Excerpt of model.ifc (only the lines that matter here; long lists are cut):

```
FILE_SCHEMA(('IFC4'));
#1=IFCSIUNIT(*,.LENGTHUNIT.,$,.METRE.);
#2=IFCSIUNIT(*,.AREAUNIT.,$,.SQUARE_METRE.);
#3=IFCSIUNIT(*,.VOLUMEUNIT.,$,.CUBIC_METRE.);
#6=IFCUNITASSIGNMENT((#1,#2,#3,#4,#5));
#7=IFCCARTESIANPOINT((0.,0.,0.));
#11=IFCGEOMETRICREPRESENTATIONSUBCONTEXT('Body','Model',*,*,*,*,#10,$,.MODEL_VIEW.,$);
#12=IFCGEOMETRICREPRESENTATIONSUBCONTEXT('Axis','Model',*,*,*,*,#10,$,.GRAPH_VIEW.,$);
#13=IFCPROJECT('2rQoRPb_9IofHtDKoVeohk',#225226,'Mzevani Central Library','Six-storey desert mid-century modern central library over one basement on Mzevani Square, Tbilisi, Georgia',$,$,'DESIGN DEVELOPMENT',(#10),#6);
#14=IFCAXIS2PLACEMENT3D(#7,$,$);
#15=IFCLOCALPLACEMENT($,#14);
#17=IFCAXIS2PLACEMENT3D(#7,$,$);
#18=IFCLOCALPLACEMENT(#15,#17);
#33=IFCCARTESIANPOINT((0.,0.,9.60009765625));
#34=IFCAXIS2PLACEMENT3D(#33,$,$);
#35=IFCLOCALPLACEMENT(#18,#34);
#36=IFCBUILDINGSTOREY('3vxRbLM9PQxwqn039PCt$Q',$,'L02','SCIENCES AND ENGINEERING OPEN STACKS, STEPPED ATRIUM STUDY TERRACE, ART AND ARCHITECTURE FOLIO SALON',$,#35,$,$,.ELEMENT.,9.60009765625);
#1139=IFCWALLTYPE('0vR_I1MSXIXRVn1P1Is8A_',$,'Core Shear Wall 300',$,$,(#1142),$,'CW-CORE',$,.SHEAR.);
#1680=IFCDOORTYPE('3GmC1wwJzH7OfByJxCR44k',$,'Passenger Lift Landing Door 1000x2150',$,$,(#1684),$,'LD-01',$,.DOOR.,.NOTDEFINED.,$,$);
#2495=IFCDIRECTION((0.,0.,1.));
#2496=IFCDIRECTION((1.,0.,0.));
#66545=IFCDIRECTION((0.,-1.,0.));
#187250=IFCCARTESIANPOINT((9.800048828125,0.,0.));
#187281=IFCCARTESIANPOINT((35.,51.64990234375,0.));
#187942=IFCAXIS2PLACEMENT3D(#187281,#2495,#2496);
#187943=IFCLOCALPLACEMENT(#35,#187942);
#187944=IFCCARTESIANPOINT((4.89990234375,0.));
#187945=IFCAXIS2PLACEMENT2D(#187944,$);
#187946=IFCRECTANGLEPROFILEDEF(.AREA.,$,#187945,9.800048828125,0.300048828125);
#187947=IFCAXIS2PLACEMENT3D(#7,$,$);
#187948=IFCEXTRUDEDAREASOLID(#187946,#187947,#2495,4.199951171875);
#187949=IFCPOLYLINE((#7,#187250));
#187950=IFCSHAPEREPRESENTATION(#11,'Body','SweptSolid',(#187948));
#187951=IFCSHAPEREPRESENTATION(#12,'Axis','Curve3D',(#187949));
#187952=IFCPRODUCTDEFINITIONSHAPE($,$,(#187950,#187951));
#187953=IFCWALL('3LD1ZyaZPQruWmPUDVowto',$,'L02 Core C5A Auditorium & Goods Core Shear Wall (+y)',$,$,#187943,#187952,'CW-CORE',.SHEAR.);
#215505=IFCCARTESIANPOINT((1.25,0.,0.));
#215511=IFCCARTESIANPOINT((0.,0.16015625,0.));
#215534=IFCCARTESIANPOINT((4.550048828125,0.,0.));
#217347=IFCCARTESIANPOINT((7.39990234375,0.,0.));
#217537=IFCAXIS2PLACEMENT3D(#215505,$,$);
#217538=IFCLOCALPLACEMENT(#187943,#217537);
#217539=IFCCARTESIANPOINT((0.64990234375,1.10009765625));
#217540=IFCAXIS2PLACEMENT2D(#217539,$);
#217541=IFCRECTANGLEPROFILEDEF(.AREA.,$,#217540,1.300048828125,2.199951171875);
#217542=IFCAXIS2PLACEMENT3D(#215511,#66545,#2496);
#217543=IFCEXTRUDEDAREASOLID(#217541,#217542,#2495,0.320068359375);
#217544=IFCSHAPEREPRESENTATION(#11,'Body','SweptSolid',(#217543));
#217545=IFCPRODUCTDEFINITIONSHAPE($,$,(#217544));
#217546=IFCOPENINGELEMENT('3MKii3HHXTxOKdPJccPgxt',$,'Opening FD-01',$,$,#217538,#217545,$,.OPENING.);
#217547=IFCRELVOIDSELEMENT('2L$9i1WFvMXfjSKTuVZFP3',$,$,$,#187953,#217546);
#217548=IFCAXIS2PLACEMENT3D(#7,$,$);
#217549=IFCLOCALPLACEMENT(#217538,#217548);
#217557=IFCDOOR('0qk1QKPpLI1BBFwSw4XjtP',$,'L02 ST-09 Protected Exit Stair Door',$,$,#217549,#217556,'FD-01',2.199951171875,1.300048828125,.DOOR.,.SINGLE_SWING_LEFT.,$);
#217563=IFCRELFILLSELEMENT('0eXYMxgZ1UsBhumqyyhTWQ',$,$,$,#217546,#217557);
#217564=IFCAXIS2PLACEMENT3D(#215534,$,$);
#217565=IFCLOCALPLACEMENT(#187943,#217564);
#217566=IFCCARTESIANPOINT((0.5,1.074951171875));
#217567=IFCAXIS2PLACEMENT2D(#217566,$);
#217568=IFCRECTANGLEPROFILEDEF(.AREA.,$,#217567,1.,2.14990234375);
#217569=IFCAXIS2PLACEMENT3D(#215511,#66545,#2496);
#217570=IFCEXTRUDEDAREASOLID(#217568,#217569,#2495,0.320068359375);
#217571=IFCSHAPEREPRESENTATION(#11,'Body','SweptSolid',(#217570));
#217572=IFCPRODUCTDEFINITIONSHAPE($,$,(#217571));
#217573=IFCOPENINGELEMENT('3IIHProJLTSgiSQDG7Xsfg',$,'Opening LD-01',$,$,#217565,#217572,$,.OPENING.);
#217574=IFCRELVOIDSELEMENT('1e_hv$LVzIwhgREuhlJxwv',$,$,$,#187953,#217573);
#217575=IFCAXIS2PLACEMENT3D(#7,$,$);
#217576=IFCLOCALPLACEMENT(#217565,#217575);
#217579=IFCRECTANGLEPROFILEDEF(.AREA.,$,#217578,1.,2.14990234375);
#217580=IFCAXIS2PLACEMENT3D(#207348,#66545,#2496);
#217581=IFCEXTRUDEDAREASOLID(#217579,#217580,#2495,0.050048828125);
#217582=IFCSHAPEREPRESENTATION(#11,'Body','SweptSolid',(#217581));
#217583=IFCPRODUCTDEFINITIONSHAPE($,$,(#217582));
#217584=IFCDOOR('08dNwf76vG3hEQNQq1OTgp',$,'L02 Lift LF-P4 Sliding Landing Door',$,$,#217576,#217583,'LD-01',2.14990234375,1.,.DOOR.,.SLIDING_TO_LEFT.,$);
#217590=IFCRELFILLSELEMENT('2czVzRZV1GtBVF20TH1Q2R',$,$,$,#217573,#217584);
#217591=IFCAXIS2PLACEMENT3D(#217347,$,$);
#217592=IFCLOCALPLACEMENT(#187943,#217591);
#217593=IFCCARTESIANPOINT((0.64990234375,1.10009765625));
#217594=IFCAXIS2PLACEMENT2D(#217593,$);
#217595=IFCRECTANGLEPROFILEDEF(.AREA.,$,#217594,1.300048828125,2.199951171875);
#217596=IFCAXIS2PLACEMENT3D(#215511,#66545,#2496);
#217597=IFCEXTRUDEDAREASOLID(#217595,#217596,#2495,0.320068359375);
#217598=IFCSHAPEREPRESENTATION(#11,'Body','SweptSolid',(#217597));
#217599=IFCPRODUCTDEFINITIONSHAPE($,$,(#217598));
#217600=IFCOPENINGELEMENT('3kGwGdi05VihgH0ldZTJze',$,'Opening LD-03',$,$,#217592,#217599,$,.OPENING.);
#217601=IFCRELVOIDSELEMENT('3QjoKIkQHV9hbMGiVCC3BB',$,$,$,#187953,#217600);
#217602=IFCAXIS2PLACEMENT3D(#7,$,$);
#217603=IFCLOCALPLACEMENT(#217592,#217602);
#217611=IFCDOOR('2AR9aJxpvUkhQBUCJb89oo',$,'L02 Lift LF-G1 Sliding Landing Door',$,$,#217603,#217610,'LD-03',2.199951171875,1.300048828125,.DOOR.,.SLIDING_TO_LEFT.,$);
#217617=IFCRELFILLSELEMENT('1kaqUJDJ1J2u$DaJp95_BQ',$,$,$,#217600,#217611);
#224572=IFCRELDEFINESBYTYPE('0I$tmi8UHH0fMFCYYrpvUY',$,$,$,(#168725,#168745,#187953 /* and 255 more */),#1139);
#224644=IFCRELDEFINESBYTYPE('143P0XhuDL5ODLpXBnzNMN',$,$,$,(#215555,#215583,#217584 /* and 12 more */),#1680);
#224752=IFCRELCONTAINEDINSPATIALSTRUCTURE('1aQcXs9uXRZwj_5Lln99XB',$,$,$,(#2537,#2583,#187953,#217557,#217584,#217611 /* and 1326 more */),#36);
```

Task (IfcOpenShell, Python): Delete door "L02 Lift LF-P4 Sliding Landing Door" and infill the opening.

```python
import ifcopenshell
import ifcopenshell.api.feature
import ifcopenshell.api.root
import ifcopenshell.geom
import ifcopenshell.util.shape

model = ifcopenshell.open("model.ifc")
settings = ifcopenshell.geom.settings()


def volume(element):
    """Net volume in cubic metres, openings subtracted."""
    shape = ifcopenshell.geom.create_shape(settings, element)
    return ifcopenshell.util.shape.get_volume(shape.geometry)


door = model.by_guid("08dNwf76vG3hEQNQq1OTgp")
opening = door.FillsVoids[0].RelatingOpeningElement
wall = opening.VoidsElements[0].RelatingBuildingElement
before = volume(wall)

ifcopenshell.api.root.remove_product(model, product=door)
ifcopenshell.api.feature.remove_feature(model, feature=opening)

after = volume(wall)

print(f"wall volume {before:.3f} -> {after:.3f} m3")

model.write("model-out.ifc")
```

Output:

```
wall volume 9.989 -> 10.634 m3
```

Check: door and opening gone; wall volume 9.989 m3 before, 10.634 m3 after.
